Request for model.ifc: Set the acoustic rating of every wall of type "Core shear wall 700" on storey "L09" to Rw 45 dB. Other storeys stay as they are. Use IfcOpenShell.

First a look at what the model holds.

```python
import ifcopenshell
import ifcopenshell.util.element

model = ifcopenshell.open("model.ifc")
print(model.schema)
storey = next(s for s in model.by_type("IfcBuildingStorey") if s.Name == "L09")
walls = [e for e in ifcopenshell.util.element.get_decomposition(storey) if e.is_a("IfcWall")]
seen = {}
for e in walls:
    element_type = ifcopenshell.util.element.get_type(e)
    key = (element_type.Name if element_type != e and element_type else None, ifcopenshell.util.element.get_pset(e, "Pset_WallCommon", "AcousticRating"))
    seen[key] = seen.get(key, 0) + 1
for (name, value), count in sorted(seen.items(), key=str):
    print(count, "x", name, "|", value)
```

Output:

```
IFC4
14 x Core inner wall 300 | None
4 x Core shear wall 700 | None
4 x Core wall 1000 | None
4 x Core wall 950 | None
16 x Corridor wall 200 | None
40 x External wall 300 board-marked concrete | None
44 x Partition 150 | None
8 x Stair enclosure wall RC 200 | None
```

```python
import ifcopenshell
import ifcopenshell.api.pset
import ifcopenshell.util.element

model = ifcopenshell.open("model.ifc")

storey = next(s for s in model.by_type("IfcBuildingStorey") if s.Name == "L09")
walls = [e for e in ifcopenshell.util.element.get_decomposition(storey) if e.is_a("IfcWall")]

count = 0
for e in walls:
    element_type = ifcopenshell.util.element.get_type(e)
    if element_type in (None, e) or element_type.Name != "Core shear wall 700":
        continue
    # add_pset returns the element's existing set when there is one.
    pset = ifcopenshell.api.pset.add_pset(model, product=e, name="Pset_WallCommon")
    ifcopenshell.api.pset.edit_pset(model, pset=pset, properties={"AcousticRating": "Rw 45 dB"})
    count += 1

print(count, "walls updated")

model.write("model-out.ifc")
```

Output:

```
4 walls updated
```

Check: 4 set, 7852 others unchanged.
